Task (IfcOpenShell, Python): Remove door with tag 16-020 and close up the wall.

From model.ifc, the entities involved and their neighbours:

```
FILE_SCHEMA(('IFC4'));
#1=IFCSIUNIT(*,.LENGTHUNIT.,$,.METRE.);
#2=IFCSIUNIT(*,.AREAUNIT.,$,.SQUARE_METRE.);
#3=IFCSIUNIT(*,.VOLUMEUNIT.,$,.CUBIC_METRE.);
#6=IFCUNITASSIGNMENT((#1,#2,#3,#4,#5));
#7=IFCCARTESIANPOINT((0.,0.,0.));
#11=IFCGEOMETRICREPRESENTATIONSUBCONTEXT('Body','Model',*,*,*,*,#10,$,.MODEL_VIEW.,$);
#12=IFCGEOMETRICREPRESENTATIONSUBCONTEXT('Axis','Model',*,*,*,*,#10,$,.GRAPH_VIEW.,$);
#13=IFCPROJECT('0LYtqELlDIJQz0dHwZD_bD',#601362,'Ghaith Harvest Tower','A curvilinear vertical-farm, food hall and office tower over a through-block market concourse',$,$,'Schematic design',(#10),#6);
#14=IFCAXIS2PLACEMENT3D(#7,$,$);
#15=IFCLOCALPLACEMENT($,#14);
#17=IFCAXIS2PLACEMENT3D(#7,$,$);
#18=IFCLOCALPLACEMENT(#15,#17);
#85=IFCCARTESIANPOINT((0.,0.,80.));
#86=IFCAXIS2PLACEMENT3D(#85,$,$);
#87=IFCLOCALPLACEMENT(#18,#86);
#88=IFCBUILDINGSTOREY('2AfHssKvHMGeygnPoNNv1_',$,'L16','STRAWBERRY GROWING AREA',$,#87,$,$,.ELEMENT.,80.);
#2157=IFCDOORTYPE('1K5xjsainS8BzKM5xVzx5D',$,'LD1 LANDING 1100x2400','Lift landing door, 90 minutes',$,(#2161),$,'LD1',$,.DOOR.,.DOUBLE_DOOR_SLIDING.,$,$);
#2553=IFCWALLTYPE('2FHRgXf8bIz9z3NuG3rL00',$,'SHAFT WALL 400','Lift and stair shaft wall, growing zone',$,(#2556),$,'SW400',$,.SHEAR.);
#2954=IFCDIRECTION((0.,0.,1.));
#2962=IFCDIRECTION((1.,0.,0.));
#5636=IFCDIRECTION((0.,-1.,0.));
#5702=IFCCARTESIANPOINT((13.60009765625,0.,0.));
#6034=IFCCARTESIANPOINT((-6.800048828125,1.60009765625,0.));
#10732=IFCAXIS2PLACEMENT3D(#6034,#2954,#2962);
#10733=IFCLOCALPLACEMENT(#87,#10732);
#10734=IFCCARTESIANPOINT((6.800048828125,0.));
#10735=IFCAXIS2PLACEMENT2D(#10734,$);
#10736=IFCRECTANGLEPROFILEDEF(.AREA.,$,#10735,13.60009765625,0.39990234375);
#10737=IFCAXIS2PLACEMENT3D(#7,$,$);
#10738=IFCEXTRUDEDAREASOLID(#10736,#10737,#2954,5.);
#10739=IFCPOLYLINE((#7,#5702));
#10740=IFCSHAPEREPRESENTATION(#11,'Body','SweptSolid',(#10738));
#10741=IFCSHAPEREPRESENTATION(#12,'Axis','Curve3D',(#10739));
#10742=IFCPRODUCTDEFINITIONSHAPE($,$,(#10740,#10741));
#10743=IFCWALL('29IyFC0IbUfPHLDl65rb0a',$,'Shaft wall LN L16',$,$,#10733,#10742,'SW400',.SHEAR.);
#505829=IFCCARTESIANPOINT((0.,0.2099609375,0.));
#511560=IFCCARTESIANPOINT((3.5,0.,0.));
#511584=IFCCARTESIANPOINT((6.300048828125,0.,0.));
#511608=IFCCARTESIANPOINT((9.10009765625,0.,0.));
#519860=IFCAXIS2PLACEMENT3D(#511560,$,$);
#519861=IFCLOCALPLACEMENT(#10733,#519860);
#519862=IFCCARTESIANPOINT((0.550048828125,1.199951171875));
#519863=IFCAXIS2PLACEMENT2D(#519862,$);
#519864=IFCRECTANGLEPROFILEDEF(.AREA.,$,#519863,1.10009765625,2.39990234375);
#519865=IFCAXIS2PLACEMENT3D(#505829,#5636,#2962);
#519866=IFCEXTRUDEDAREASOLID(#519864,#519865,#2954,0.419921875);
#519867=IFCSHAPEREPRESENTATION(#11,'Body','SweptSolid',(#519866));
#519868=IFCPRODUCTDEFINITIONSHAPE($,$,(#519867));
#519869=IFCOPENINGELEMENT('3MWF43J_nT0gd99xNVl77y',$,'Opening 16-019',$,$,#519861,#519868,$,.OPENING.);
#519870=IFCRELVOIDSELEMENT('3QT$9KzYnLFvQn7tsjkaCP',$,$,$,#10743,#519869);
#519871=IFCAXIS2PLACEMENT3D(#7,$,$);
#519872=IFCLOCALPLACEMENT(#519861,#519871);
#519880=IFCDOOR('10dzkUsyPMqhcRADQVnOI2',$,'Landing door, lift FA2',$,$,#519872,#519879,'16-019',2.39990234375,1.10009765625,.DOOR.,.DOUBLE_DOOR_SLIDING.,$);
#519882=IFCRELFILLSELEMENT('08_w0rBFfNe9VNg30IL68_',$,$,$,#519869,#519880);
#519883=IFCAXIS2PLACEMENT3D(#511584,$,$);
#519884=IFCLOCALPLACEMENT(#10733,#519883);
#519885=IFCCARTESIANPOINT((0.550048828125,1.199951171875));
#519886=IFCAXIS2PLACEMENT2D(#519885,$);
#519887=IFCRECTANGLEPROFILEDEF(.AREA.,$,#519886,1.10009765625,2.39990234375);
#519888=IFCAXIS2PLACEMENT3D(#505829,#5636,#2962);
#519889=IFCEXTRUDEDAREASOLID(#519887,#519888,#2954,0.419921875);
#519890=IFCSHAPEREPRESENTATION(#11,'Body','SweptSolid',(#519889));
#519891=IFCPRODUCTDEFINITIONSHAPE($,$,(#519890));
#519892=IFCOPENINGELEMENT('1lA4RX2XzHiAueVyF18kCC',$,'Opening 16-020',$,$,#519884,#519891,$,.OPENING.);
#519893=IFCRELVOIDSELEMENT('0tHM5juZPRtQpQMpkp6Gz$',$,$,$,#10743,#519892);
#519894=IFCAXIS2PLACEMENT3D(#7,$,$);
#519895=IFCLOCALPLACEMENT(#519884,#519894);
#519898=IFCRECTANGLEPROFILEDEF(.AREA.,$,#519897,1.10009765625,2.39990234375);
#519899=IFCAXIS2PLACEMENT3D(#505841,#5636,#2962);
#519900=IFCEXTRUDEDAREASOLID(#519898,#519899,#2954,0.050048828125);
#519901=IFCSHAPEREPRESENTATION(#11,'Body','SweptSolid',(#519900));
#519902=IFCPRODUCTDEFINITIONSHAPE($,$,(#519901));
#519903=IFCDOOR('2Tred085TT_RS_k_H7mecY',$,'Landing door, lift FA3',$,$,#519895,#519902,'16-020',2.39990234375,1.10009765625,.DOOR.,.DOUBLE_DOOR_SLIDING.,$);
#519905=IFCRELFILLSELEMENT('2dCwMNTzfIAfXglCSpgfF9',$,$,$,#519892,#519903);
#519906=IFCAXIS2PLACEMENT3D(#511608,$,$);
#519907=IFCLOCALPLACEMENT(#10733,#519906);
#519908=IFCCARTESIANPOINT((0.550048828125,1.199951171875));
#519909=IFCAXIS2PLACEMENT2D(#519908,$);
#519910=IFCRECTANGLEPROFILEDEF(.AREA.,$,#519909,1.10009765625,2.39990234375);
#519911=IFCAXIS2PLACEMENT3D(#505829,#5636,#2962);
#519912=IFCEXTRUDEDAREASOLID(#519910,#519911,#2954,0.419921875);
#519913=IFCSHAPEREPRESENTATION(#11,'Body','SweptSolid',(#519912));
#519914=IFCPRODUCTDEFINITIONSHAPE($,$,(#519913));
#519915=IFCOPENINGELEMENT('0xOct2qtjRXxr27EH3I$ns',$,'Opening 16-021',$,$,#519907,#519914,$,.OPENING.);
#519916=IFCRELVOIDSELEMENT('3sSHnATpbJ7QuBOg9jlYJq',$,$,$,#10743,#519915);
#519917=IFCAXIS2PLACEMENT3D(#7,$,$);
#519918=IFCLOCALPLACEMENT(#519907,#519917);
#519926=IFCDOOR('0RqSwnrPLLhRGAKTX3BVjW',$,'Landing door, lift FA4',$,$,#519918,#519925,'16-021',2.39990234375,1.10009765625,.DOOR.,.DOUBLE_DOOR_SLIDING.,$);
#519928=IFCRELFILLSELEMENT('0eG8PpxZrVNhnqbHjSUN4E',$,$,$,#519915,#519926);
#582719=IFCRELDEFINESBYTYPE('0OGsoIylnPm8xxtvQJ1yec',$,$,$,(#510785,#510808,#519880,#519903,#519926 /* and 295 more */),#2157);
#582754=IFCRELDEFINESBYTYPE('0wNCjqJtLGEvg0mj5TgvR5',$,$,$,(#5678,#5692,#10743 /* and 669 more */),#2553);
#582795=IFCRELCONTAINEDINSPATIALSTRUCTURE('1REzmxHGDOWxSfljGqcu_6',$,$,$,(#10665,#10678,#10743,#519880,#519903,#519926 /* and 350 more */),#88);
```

```python
import ifcopenshell
import ifcopenshell.api.feature
import ifcopenshell.api.root
import ifcopenshell.geom
import ifcopenshell.util.shape

model = ifcopenshell.open("model.ifc")
settings = ifcopenshell.geom.settings()


def volume(element):
    """Net volume in cubic metres, openings subtracted."""
    shape = ifcopenshell.geom.create_shape(settings, element)
    return ifcopenshell.util.shape.get_volume(shape.geometry)


door = model.by_id(519903)
opening = door.FillsVoids[0].RelatingOpeningElement
wall = opening.VoidsElements[0].RelatingBuildingElement
before = volume(wall)

ifcopenshell.api.root.remove_product(model, product=door)
ifcopenshell.api.feature.remove_feature(model, feature=opening)

after = volume(wall)

print(f"wall volume {before:.3f} -> {after:.3f} m3")

model.write("model-out.ifc")
```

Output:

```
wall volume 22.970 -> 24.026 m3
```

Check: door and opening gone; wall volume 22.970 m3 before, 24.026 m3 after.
